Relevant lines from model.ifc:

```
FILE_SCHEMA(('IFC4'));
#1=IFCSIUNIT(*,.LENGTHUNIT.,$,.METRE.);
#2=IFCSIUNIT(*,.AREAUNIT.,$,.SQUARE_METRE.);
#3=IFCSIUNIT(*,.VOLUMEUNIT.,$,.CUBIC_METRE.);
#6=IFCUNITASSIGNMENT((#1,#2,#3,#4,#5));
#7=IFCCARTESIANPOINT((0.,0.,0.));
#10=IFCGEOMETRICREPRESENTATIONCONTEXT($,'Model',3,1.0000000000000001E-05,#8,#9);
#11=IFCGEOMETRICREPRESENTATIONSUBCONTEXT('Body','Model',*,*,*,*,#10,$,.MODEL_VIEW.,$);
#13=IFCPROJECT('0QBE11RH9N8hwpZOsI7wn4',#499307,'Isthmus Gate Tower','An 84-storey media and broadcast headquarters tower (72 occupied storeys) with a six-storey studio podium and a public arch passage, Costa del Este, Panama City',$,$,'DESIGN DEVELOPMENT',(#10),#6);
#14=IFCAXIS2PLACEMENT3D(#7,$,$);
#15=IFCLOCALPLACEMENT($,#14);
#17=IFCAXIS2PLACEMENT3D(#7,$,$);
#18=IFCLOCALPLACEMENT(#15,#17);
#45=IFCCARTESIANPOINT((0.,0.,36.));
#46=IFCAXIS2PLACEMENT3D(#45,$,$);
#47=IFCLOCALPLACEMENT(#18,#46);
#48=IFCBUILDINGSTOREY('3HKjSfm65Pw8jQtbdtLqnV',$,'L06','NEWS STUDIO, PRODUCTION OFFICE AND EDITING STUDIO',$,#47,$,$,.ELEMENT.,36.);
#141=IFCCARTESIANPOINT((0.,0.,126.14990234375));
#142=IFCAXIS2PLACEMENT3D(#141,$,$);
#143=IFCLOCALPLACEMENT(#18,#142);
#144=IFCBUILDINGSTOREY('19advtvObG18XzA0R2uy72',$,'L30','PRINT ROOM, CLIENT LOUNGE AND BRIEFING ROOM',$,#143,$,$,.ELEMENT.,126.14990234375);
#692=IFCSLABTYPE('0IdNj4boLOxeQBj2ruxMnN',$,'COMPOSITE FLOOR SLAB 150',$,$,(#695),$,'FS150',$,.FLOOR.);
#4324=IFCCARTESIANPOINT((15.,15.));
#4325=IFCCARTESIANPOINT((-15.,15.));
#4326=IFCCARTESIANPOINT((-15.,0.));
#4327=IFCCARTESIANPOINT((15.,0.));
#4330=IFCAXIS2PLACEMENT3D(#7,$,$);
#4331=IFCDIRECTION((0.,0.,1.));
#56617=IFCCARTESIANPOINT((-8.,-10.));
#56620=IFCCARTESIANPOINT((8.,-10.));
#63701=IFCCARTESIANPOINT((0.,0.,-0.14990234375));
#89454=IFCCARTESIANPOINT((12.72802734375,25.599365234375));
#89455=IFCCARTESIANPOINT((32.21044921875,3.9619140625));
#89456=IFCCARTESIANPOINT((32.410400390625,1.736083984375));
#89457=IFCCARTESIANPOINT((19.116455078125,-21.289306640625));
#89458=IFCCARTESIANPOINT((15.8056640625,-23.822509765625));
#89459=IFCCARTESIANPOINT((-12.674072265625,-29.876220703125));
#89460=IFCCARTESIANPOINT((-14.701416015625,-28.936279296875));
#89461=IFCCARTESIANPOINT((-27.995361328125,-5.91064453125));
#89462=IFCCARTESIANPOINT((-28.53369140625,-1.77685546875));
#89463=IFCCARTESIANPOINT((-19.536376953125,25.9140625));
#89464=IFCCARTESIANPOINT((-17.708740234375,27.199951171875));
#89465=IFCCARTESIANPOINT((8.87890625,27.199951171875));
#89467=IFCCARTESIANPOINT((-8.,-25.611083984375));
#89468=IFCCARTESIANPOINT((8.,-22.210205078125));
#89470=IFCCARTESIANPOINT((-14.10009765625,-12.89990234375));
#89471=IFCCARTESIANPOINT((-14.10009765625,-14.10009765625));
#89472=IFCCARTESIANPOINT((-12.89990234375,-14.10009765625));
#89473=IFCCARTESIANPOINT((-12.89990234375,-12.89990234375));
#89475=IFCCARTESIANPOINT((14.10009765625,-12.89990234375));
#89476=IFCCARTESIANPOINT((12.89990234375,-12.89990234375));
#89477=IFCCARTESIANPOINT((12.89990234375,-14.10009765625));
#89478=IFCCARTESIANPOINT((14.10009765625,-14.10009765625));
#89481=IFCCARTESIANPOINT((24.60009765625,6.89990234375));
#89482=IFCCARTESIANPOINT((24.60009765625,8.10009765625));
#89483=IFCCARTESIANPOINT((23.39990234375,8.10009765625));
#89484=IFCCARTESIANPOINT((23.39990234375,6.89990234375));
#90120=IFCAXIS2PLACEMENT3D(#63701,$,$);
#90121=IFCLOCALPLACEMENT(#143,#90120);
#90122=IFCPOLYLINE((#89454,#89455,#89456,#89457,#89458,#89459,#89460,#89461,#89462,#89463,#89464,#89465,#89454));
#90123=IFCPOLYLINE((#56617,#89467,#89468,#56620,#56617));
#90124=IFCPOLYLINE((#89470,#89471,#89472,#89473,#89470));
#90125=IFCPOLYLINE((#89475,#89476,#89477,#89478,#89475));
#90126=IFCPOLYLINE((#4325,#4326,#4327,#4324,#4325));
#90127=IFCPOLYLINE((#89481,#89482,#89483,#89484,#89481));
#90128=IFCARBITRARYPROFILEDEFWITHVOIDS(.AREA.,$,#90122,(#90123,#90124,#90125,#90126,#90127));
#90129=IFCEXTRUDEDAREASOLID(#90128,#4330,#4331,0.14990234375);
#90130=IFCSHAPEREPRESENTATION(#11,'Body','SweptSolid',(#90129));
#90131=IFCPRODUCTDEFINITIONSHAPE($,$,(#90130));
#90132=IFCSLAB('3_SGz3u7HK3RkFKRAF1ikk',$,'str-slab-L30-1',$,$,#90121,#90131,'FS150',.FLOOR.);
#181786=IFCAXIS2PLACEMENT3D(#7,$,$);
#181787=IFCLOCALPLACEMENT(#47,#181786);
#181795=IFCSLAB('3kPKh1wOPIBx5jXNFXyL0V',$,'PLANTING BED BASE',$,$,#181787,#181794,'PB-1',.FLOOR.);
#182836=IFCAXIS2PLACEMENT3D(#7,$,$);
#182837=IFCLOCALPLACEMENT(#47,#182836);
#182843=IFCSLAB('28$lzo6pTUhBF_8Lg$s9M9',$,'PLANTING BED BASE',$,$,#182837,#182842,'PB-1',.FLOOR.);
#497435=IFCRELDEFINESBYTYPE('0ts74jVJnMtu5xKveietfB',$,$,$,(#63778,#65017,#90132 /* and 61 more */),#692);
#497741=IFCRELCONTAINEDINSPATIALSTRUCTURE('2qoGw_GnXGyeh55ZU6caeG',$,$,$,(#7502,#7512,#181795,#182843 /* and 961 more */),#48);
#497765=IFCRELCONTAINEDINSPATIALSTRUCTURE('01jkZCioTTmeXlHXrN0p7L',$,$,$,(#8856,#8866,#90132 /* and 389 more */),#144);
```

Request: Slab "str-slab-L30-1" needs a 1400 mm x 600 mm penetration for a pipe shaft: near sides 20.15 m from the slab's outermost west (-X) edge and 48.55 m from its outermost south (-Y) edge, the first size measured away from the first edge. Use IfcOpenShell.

```python
import numpy as np
import ifcopenshell
import ifcopenshell.api.feature
import ifcopenshell.api.geometry
import ifcopenshell.api.root
import ifcopenshell.geom
import ifcopenshell.util.placement
import ifcopenshell.util.representation
import ifcopenshell.util.shape
import ifcopenshell.util.unit

model = ifcopenshell.open("model.ifc")
unit_scale = ifcopenshell.util.unit.calculate_unit_scale(model)
settings = ifcopenshell.geom.settings()


def volume(element):
    """Net volume in cubic metres, openings subtracted."""
    shape = ifcopenshell.geom.create_shape(settings, element)
    return ifcopenshell.util.shape.get_volume(shape.geometry)


slab = model.by_id(90132)
before = volume(slab)

# Extent in the slab's own axes, in metres. The edges named are its -X and -Y sides.
slab_shape = ifcopenshell.geom.create_shape(settings, slab)
vertices = ifcopenshell.util.shape.get_vertices(slab_shape.geometry)
x_min, y_min, bottom = vertices.min(axis=0)
top = vertices[:, 2].max()

opening = ifcopenshell.api.root.create_entity(model, ifc_class="IfcOpeningElement", name="Pipe shaft opening", predefined_type="OPENING")
context = ifcopenshell.util.representation.get_context(model, "Model", "Body", "MODEL_VIEW")
width, depth = 1.4, 0.6
outline = [(0.0, 0.0), (width, 0.0), (width, depth), (0.0, depth), (0.0, 0.0)]
# Overshoot both faces by 50 mm so the cut is clean.
shape = ifcopenshell.api.geometry.add_slab_representation(
    model, context=context, depth=top - bottom + 0.1, polyline=outline
)
ifcopenshell.api.geometry.assign_representation(model, product=opening, representation=shape)

matrix = ifcopenshell.util.placement.get_local_placement(slab.ObjectPlacement)
matrix[:, 3] = matrix @ np.append(np.array([x_min + 20.15, y_min + 48.55, bottom - 0.05]) / unit_scale, 1.0)
ifcopenshell.api.geometry.edit_object_placement(model, product=opening, matrix=matrix, is_si=False)
ifcopenshell.api.feature.add_feature(model, feature=opening, element=slab)

after = volume(slab)

print(f"slab volume {before:.3f} -> {after:.3f} m3")

model.write("model_v2.ifc")
```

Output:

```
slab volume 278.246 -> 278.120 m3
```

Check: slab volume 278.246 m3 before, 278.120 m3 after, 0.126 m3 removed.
